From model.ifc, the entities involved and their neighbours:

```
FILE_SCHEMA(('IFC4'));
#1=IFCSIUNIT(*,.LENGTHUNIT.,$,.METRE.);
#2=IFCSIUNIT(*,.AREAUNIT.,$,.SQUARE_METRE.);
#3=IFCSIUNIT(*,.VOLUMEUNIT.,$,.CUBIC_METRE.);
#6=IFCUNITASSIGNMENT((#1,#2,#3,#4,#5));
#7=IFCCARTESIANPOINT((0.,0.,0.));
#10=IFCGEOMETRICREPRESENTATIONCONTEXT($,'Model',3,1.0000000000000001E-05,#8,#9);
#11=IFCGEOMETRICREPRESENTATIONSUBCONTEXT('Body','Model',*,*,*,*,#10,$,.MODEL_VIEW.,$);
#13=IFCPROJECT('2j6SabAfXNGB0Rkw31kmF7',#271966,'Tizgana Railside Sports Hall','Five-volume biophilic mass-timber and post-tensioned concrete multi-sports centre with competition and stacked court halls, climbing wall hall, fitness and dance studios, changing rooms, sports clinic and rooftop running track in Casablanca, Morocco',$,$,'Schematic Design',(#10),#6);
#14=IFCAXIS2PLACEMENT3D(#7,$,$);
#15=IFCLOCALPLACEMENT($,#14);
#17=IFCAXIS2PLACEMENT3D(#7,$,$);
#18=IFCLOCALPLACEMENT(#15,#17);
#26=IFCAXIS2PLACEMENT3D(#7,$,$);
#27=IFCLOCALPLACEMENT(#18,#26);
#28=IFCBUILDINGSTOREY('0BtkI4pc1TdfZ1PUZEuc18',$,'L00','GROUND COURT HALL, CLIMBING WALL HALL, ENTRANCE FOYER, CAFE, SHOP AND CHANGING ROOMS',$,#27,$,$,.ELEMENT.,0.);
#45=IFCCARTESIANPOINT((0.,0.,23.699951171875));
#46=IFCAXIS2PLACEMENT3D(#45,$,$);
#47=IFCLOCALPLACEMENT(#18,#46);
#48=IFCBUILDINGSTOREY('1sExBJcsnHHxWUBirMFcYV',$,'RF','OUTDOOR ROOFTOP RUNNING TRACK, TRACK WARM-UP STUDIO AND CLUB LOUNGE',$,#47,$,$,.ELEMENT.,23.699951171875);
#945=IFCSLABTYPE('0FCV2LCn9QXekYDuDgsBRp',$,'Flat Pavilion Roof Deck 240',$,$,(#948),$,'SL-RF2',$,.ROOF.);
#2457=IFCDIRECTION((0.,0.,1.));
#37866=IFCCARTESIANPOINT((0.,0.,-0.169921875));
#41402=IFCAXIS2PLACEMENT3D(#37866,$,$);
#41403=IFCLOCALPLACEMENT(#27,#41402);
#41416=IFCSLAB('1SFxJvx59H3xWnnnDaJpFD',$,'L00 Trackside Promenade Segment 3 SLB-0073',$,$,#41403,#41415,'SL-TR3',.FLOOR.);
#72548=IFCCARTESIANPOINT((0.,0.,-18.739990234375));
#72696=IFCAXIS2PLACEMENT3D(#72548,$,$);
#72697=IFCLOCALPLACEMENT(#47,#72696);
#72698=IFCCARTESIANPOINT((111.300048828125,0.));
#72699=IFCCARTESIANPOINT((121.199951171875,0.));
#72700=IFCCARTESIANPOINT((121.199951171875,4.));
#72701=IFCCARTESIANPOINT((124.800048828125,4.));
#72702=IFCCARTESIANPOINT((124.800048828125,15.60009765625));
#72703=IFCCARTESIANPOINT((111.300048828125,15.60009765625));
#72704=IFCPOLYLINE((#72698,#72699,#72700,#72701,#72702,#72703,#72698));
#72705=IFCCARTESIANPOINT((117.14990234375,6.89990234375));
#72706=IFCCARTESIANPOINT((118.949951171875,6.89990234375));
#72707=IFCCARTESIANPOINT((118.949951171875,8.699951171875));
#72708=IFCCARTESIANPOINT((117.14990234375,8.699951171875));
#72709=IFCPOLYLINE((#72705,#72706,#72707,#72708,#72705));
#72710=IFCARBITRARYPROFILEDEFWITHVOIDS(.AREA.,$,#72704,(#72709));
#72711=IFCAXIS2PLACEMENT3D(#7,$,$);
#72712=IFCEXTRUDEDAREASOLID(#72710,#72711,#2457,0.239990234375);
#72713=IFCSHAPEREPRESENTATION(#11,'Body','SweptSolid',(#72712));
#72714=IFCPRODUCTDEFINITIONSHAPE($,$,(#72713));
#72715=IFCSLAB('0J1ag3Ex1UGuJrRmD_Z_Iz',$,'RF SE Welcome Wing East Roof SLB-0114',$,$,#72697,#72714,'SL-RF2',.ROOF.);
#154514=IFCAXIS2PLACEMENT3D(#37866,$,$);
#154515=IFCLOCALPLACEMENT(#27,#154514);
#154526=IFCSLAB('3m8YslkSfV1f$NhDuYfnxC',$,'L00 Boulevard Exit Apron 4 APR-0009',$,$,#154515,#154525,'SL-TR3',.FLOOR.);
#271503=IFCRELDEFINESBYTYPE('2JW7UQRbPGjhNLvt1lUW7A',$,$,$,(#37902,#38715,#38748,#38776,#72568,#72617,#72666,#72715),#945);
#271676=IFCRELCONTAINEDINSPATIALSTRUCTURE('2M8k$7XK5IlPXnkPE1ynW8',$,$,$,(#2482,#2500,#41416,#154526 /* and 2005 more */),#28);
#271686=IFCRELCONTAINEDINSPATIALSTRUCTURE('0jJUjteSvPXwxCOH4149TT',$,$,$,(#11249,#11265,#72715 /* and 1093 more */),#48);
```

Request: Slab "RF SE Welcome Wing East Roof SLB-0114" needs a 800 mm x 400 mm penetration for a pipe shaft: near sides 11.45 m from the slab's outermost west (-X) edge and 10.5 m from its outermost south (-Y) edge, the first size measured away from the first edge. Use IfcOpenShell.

```python
import numpy as np
import ifcopenshell
import ifcopenshell.api.feature
import ifcopenshell.api.geometry
import ifcopenshell.api.root
import ifcopenshell.geom
import ifcopenshell.util.placement
import ifcopenshell.util.representation
import ifcopenshell.util.shape
import ifcopenshell.util.unit

model = ifcopenshell.open("model.ifc")
unit_scale = ifcopenshell.util.unit.calculate_unit_scale(model)
settings = ifcopenshell.geom.settings()


def volume(element):
    """Net volume in cubic metres, openings subtracted."""
    shape = ifcopenshell.geom.create_shape(settings, element)
    return ifcopenshell.util.shape.get_volume(shape.geometry)


slab = model.by_guid("0J1ag3Ex1UGuJrRmD_Z_Iz")
before = volume(slab)

# Extent in the slab's own axes, in metres. The edges named are its -X and -Y sides.
slab_shape = ifcopenshell.geom.create_shape(settings, slab)
vertices = ifcopenshell.util.shape.get_vertices(slab_shape.geometry)
x_min, y_min, bottom = vertices.min(axis=0)
top = vertices[:, 2].max()

opening = ifcopenshell.api.root.create_entity(model, ifc_class="IfcOpeningElement", name="Pipe shaft opening", predefined_type="OPENING")
context = ifcopenshell.util.representation.get_context(model, "Model", "Body", "MODEL_VIEW")
width, depth = 0.8, 0.4
outline = [(0.0, 0.0), (width, 0.0), (width, depth), (0.0, depth), (0.0, 0.0)]
# Overshoot both faces by 50 mm so the cut is clean.
shape = ifcopenshell.api.geometry.add_slab_representation(
    model, context=context, depth=top - bottom + 0.1, polyline=outline
)
ifcopenshell.api.geometry.assign_representation(model, product=opening, representation=shape)

matrix = ifcopenshell.util.placement.get_local_placement(slab.ObjectPlacement)
matrix[:, 3] = matrix @ np.append(np.array([x_min + 11.45, y_min + 10.5, bottom - 0.05]) / unit_scale, 1.0)
ifcopenshell.api.geometry.edit_object_placement(model, product=opening, matrix=matrix, is_si=False)
ifcopenshell.api.feature.add_feature(model, feature=opening, element=slab)

after = volume(slab)

print(f"slab volume {before:.3f} -> {after:.3f} m3")

model.write("model_edited.ifc")
```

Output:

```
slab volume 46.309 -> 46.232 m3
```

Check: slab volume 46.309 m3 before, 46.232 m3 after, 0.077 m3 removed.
